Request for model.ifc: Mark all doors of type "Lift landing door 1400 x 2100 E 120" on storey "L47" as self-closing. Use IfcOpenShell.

First a look at what the model holds.

```python
import ifcopenshell
import ifcopenshell.util.element

model = ifcopenshell.open("model.ifc")
print(model.schema)
storey = next(s for s in model.by_type("IfcBuildingStorey") if s.Name == "L47")
doors = [e for e in ifcopenshell.util.element.get_decomposition(storey) if e.is_a("IfcDoor")]
seen = {}
for e in doors:
    element_type = ifcopenshell.util.element.get_type(e)
    key = (element_type.Name if element_type != e and element_type else None, ifcopenshell.util.element.get_pset(e, "Pset_DoorCommon", "SelfClosing"))
    seen[key] = seen.get(key, 0) + 1
for (name, value), count in sorted(seen.items(), key=str):
    print(count, "x", name, "|", value)
```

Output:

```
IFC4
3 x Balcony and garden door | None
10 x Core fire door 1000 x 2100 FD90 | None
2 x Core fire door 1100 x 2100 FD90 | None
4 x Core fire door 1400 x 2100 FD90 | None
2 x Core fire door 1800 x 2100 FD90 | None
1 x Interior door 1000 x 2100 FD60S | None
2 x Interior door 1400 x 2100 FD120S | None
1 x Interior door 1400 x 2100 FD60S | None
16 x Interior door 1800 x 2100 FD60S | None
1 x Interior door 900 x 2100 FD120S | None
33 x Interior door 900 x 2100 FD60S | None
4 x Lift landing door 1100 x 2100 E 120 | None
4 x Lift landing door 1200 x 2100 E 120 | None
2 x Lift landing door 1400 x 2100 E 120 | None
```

```python
import ifcopenshell
import ifcopenshell.api.pset
import ifcopenshell.util.element

model = ifcopenshell.open("model.ifc")

storey = next(s for s in model.by_type("IfcBuildingStorey") if s.Name == "L47")
doors = [e for e in ifcopenshell.util.element.get_decomposition(storey) if e.is_a("IfcDoor")]

count = 0
for e in doors:
    element_type = ifcopenshell.util.element.get_type(e)
    if element_type in (None, e) or element_type.Name != "Lift landing door 1400 x 2100 E 120":
        continue
    # add_pset returns the element's existing set when there is one.
    pset = ifcopenshell.api.pset.add_pset(model, product=e, name="Pset_DoorCommon")
    ifcopenshell.api.pset.edit_pset(model, pset=pset, properties={"SelfClosing": True})
    count += 1

print(count, "doors updated")

model.write("model_edited.ifc")
```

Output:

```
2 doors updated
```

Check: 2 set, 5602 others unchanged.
